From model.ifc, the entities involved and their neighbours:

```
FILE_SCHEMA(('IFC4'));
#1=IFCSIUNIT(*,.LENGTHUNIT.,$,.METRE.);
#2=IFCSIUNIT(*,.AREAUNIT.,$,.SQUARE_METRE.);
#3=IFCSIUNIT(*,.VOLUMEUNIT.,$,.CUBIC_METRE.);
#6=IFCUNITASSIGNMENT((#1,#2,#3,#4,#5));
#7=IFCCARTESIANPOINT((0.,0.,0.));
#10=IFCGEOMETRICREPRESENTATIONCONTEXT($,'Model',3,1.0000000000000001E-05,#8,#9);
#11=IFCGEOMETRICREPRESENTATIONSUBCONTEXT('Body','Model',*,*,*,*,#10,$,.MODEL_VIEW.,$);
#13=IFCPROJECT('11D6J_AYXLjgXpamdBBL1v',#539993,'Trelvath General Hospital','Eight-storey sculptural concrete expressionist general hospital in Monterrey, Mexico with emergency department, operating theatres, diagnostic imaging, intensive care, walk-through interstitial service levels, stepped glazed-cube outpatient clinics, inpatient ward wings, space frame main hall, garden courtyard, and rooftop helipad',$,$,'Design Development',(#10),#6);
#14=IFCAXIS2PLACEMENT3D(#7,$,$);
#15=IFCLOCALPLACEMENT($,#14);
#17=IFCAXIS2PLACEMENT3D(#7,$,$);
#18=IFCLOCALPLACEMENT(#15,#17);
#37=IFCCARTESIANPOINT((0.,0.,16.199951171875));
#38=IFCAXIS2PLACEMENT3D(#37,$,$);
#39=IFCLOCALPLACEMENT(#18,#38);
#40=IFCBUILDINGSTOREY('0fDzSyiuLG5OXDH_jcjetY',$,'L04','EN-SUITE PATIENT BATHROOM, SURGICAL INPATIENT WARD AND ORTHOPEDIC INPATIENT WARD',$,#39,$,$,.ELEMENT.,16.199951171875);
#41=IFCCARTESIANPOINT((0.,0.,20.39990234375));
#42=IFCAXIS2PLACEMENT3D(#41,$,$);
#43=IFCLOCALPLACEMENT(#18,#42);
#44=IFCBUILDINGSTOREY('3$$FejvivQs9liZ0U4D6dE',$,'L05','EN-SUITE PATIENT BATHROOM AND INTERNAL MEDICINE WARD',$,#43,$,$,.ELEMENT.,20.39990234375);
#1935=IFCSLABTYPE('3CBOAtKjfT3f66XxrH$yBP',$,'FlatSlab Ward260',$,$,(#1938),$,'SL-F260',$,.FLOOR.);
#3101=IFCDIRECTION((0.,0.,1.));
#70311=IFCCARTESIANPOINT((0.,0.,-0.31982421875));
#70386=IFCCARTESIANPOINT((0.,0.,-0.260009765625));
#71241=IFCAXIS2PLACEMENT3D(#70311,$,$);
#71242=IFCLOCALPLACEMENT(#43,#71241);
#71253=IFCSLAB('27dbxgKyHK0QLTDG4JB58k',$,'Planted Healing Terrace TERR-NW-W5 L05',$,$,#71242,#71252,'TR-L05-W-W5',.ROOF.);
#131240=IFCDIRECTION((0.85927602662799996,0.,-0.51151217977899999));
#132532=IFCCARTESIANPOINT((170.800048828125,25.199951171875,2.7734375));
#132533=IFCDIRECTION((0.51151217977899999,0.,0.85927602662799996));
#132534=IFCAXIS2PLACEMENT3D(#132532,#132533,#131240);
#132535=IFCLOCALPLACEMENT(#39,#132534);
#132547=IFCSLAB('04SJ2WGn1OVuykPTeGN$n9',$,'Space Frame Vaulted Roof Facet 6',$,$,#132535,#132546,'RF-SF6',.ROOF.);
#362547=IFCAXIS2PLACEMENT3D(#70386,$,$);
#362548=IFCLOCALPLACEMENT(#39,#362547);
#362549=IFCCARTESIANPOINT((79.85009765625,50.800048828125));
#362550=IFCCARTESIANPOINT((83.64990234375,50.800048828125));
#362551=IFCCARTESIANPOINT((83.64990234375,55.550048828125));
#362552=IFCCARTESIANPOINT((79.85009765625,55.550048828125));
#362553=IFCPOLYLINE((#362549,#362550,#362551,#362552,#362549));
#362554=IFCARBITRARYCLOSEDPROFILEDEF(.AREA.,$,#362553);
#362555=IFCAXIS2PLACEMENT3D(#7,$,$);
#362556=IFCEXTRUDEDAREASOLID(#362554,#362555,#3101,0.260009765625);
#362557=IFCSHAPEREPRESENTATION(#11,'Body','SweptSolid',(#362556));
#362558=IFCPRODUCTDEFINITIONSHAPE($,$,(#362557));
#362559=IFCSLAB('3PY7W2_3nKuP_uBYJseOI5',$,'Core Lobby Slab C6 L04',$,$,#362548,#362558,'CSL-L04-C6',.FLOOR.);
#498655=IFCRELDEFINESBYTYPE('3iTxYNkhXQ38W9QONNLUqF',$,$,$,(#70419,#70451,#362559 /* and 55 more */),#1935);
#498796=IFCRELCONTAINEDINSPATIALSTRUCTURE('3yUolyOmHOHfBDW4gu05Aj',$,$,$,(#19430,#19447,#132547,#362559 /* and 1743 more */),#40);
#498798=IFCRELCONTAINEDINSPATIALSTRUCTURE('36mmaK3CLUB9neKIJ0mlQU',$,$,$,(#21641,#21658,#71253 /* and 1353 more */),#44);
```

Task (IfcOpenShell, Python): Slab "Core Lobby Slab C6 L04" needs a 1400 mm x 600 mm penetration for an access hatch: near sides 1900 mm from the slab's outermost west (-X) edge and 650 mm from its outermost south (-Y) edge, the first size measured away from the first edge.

```python
import numpy as np
import ifcopenshell
import ifcopenshell.api.feature
import ifcopenshell.api.geometry
import ifcopenshell.api.root
import ifcopenshell.geom
import ifcopenshell.util.placement
import ifcopenshell.util.representation
import ifcopenshell.util.shape
import ifcopenshell.util.unit

model = ifcopenshell.open("model.ifc")
unit_scale = ifcopenshell.util.unit.calculate_unit_scale(model)
settings = ifcopenshell.geom.settings()


def volume(element):
    """Net volume in cubic metres, openings subtracted."""
    shape = ifcopenshell.geom.create_shape(settings, element)
    return ifcopenshell.util.shape.get_volume(shape.geometry)


slab = model.by_id(362559)
before = volume(slab)

# Extent in the slab's own axes, in metres. The edges named are its -X and -Y sides.
slab_shape = ifcopenshell.geom.create_shape(settings, slab)
vertices = ifcopenshell.util.shape.get_vertices(slab_shape.geometry)
x_min, y_min, bottom = vertices.min(axis=0)
top = vertices[:, 2].max()

opening = ifcopenshell.api.root.create_entity(model, ifc_class="IfcOpeningElement", name="Access hatch opening", predefined_type="OPENING")
context = ifcopenshell.util.representation.get_context(model, "Model", "Body", "MODEL_VIEW")
width, depth = 1.4, 0.6
outline = [(0.0, 0.0), (width, 0.0), (width, depth), (0.0, depth), (0.0, 0.0)]
# Overshoot both faces by 50 mm so the cut is clean.
shape = ifcopenshell.api.geometry.add_slab_representation(
    model, context=context, depth=top - bottom + 0.1, polyline=outline
)
ifcopenshell.api.geometry.assign_representation(model, product=opening, representation=shape)

matrix = ifcopenshell.util.placement.get_local_placement(slab.ObjectPlacement)
matrix[:, 3] = matrix @ np.append(np.array([x_min + 1.9, y_min + 0.65, bottom - 0.05]) / unit_scale, 1.0)
ifcopenshell.api.geometry.edit_object_placement(model, product=opening, matrix=matrix, is_si=False)
ifcopenshell.api.feature.add_feature(model, feature=opening, element=slab)

after = volume(slab)

print(f"slab volume {before:.3f} -> {after:.3f} m3")

model.write("model_v2.ifc")
```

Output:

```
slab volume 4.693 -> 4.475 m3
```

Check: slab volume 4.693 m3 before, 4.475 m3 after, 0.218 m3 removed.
